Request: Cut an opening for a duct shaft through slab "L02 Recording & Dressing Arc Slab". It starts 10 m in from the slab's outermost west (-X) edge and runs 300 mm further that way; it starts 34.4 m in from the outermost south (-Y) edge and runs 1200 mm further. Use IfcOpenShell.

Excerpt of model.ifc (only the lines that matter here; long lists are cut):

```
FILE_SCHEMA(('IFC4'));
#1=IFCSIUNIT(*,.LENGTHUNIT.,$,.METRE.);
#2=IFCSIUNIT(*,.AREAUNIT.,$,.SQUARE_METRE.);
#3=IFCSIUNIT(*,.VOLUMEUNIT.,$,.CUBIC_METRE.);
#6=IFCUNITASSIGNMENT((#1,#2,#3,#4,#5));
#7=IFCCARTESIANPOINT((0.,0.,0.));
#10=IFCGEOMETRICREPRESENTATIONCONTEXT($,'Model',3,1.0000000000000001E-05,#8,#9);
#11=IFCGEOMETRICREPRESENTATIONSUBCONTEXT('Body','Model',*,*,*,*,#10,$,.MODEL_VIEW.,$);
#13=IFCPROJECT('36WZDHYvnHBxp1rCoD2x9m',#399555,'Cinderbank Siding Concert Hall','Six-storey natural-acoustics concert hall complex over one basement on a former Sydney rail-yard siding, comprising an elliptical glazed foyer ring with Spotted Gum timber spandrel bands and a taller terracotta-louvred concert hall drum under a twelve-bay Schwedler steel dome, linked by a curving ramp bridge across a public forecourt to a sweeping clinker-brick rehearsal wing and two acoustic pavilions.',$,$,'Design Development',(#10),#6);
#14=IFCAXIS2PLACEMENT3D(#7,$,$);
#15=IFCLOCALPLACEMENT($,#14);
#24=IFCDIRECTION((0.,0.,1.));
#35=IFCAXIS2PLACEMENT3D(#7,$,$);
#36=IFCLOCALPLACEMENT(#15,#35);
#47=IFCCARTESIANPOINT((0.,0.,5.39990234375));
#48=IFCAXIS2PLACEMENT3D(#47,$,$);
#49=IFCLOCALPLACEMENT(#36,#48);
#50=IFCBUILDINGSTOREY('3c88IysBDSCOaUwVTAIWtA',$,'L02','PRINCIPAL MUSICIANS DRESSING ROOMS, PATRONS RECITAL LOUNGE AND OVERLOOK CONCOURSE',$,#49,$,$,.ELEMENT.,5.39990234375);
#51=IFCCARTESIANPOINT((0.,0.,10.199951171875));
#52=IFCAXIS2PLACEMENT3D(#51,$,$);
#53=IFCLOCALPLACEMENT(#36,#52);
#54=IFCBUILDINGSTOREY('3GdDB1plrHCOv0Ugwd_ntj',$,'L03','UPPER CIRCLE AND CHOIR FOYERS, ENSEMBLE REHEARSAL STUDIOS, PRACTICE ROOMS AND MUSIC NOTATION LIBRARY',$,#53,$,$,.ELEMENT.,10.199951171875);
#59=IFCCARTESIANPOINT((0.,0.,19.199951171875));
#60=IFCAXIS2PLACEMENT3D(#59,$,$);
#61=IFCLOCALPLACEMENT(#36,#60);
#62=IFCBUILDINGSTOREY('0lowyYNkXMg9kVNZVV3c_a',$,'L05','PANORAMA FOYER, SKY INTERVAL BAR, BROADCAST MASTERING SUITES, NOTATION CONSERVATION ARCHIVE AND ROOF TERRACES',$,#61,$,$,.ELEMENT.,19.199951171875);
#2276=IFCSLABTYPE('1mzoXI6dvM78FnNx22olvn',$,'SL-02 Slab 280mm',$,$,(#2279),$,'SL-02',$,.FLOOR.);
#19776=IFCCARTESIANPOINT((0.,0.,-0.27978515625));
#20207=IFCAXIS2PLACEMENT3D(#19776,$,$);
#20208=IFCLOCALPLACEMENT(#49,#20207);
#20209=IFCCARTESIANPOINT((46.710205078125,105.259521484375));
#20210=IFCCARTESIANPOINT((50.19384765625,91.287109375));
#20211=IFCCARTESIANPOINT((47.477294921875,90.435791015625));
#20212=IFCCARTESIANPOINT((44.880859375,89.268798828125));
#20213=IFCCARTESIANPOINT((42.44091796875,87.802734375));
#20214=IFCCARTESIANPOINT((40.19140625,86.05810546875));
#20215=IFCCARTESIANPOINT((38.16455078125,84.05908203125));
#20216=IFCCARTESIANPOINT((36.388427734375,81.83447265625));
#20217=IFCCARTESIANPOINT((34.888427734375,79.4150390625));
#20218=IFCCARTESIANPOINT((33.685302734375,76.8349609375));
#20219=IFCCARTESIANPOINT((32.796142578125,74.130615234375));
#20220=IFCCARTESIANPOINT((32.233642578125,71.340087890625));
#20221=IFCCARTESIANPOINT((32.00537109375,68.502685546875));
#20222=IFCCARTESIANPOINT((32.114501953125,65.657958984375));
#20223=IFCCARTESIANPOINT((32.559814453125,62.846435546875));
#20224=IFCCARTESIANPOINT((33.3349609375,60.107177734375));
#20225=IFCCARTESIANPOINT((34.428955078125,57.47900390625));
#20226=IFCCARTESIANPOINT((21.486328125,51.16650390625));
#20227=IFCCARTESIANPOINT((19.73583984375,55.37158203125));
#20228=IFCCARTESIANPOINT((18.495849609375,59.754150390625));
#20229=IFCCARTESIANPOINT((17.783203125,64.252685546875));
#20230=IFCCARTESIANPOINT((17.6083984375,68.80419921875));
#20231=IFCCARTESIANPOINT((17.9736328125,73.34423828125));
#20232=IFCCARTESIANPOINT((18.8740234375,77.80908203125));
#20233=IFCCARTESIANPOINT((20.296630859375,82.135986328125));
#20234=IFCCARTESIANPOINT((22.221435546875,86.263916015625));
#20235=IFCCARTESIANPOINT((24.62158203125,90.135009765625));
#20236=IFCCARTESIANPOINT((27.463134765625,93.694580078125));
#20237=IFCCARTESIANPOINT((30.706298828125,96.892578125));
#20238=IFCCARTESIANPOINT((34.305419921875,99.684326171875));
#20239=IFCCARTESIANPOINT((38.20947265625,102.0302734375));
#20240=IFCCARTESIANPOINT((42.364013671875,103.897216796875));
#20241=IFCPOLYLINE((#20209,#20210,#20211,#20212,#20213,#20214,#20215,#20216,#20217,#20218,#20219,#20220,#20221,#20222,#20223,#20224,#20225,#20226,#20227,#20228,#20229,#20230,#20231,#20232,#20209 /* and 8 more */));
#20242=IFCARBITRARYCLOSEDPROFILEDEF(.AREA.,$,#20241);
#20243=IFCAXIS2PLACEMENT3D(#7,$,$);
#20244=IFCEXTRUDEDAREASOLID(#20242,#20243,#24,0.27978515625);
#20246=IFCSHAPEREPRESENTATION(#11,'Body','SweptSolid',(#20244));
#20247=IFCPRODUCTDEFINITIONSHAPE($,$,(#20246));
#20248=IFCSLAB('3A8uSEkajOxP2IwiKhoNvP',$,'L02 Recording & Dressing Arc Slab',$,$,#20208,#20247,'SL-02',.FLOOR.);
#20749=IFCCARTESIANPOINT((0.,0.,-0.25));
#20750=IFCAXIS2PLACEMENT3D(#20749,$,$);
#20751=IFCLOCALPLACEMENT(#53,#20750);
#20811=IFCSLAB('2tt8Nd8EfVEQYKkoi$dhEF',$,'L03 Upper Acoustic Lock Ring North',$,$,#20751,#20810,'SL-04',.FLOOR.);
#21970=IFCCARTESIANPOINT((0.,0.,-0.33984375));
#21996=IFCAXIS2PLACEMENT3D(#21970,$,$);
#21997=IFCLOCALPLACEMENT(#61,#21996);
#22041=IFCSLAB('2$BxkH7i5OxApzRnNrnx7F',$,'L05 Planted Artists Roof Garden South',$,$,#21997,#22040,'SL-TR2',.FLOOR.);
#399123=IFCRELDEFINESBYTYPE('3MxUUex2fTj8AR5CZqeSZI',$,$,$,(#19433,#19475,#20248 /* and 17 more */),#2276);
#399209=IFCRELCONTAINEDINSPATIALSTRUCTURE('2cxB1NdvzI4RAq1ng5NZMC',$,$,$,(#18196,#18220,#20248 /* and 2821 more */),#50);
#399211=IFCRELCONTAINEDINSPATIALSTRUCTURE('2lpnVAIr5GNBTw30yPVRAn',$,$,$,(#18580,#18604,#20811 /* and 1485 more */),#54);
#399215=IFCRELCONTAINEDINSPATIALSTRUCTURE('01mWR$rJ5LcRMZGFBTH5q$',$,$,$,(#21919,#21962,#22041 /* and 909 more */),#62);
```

```python
import numpy as np
import ifcopenshell
import ifcopenshell.api.feature
import ifcopenshell.api.geometry
import ifcopenshell.api.root
import ifcopenshell.geom
import ifcopenshell.util.placement
import ifcopenshell.util.representation
import ifcopenshell.util.shape
import ifcopenshell.util.unit

model = ifcopenshell.open("model.ifc")
unit_scale = ifcopenshell.util.unit.calculate_unit_scale(model)
settings = ifcopenshell.geom.settings()


def volume(element):
    """Net volume in cubic metres, openings subtracted."""
    shape = ifcopenshell.geom.create_shape(settings, element)
    return ifcopenshell.util.shape.get_volume(shape.geometry)


slab = model.by_guid("3A8uSEkajOxP2IwiKhoNvP")
before = volume(slab)

# Extent in the slab's own axes, in metres. The edges named are its -X and -Y sides.
slab_shape = ifcopenshell.geom.create_shape(settings, slab)
vertices = ifcopenshell.util.shape.get_vertices(slab_shape.geometry)
x_min, y_min, bottom = vertices.min(axis=0)
top = vertices[:, 2].max()

opening = ifcopenshell.api.root.create_entity(model, ifc_class="IfcOpeningElement", name="Duct shaft opening", predefined_type="OPENING")
context = ifcopenshell.util.representation.get_context(model, "Model", "Body", "MODEL_VIEW")
width, depth = 0.3, 1.2
outline = [(0.0, 0.0), (width, 0.0), (width, depth), (0.0, depth), (0.0, 0.0)]
# Overshoot both faces by 50 mm so the cut is clean.
shape = ifcopenshell.api.geometry.add_slab_representation(
    model, context=context, depth=top - bottom + 0.1, polyline=outline
)
ifcopenshell.api.geometry.assign_representation(model, product=opening, representation=shape)

matrix = ifcopenshell.util.placement.get_local_placement(slab.ObjectPlacement)
matrix[:, 3] = matrix @ np.append(np.array([x_min + 10, y_min + 34.4, bottom - 0.05]) / unit_scale, 1.0)
ifcopenshell.api.geometry.edit_object_placement(model, product=opening, matrix=matrix, is_si=False)
ifcopenshell.api.feature.add_feature(model, feature=opening, element=slab)

after = volume(slab)

print(f"slab volume {before:.3f} -> {after:.3f} m3")

model.write("model_edited.ifc")
```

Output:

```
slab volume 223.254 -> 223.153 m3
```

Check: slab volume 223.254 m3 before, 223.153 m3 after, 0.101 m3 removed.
